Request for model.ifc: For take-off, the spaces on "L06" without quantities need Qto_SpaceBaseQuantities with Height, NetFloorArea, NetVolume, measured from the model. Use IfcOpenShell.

First a look at what the model holds.

```python
import ifcopenshell
import ifcopenshell.util.element
import ifcopenshell.util.unit

model = ifcopenshell.open("model.ifc")
print(model.schema)
for unit_type in ("LENGTHUNIT", "AREAUNIT", "VOLUMEUNIT"):
    print(unit_type, ifcopenshell.util.unit.calculate_unit_scale(model, unit_type))
storey = next(s for s in model.by_type("IfcBuildingStorey") if s.Name == "L06")
spaces = [e for e in ifcopenshell.util.element.get_decomposition(storey) if e.is_a("IfcSpace")]
for e in sorted(spaces, key=lambda e: e.id()):
    print(e.id(), e.is_a(), e.Name, list(ifcopenshell.util.element.get_psets(e, qtos_only=True)), sep=" | ")
```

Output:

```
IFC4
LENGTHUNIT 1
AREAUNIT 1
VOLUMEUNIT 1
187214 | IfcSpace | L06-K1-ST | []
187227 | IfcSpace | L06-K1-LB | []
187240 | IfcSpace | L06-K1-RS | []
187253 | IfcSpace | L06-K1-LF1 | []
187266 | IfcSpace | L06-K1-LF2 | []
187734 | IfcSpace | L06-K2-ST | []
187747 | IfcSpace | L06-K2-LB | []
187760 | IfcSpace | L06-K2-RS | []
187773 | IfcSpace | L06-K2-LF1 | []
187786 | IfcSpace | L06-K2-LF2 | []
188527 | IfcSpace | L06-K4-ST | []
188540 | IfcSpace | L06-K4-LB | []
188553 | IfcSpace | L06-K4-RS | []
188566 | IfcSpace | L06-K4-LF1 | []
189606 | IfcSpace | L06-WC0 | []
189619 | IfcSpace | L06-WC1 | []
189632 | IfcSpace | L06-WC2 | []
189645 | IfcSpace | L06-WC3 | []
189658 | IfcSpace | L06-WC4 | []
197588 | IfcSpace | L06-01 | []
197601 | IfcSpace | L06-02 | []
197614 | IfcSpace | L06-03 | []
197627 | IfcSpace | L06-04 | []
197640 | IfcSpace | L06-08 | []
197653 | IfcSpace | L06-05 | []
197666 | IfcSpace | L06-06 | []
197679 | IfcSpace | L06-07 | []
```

```python
import ifcopenshell
import ifcopenshell.api.pset
import ifcopenshell.geom
import ifcopenshell.util.element
import ifcopenshell.util.shape
import ifcopenshell.util.unit

model = ifcopenshell.open("model.ifc")
unit_scale = ifcopenshell.util.unit.calculate_unit_scale(model)
area_scale = ifcopenshell.util.unit.calculate_unit_scale(model, "AREAUNIT")
volume_scale = ifcopenshell.util.unit.calculate_unit_scale(model, "VOLUMEUNIT")
settings = ifcopenshell.geom.settings()

storey = next(s for s in model.by_type("IfcBuildingStorey") if s.Name == "L06")
spaces = [e for e in ifcopenshell.util.element.get_decomposition(storey) if e.is_a("IfcSpace")]

for e in sorted(spaces, key=lambda e: e.id()):
    if ifcopenshell.util.element.get_psets(e, qtos_only=True, should_inherit=False):
        continue
    # Geometry comes back in metres, in the element's own axes.
    shape = ifcopenshell.geom.create_shape(settings, e)
    values = {
        "Height": ifcopenshell.util.shape.get_z(shape.geometry) / unit_scale,
        "NetFloorArea": ifcopenshell.util.shape.get_footprint_area(shape.geometry) / area_scale,
        "NetVolume": ifcopenshell.util.shape.get_volume(shape.geometry) / volume_scale,
    }
    qto = ifcopenshell.api.pset.add_qto(model, product=e, name="Qto_SpaceBaseQuantities")
    ifcopenshell.api.pset.edit_qto(model, qto=qto, properties=values)
    print(e.id(), {k: round(v, 3) for k, v in values.items()})

model.write("model-out.ifc")
```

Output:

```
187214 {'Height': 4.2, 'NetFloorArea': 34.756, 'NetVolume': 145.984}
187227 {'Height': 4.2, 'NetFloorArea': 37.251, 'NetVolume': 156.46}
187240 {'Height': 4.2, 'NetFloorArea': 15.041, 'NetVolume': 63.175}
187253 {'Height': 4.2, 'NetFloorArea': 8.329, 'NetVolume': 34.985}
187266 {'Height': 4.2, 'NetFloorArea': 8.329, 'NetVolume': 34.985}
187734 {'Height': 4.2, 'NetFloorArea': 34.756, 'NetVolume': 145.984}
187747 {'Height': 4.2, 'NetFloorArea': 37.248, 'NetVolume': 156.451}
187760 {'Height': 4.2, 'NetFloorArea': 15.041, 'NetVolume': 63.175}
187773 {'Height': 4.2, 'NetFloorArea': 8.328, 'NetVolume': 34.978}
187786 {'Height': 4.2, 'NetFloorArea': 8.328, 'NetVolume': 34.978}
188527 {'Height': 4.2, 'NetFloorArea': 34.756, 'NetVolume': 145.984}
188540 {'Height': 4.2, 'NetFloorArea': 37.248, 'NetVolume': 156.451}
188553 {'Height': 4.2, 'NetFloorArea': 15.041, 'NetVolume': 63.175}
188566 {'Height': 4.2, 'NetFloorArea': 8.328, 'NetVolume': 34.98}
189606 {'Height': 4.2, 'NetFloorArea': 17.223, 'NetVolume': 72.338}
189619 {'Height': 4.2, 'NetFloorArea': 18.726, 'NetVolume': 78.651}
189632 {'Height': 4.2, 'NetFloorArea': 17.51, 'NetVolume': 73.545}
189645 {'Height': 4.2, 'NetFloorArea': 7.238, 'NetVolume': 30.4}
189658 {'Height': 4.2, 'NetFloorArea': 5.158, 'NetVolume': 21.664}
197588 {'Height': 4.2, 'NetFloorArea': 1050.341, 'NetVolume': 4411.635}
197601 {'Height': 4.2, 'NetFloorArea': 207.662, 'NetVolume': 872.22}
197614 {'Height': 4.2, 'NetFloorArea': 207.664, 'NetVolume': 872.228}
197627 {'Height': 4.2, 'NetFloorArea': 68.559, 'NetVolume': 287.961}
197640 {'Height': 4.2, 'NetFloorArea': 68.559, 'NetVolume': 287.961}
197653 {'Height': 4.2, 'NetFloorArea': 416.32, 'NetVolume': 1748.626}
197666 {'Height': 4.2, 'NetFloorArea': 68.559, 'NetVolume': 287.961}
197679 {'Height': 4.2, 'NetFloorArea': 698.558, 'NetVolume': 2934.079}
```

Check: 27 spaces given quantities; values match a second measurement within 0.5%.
